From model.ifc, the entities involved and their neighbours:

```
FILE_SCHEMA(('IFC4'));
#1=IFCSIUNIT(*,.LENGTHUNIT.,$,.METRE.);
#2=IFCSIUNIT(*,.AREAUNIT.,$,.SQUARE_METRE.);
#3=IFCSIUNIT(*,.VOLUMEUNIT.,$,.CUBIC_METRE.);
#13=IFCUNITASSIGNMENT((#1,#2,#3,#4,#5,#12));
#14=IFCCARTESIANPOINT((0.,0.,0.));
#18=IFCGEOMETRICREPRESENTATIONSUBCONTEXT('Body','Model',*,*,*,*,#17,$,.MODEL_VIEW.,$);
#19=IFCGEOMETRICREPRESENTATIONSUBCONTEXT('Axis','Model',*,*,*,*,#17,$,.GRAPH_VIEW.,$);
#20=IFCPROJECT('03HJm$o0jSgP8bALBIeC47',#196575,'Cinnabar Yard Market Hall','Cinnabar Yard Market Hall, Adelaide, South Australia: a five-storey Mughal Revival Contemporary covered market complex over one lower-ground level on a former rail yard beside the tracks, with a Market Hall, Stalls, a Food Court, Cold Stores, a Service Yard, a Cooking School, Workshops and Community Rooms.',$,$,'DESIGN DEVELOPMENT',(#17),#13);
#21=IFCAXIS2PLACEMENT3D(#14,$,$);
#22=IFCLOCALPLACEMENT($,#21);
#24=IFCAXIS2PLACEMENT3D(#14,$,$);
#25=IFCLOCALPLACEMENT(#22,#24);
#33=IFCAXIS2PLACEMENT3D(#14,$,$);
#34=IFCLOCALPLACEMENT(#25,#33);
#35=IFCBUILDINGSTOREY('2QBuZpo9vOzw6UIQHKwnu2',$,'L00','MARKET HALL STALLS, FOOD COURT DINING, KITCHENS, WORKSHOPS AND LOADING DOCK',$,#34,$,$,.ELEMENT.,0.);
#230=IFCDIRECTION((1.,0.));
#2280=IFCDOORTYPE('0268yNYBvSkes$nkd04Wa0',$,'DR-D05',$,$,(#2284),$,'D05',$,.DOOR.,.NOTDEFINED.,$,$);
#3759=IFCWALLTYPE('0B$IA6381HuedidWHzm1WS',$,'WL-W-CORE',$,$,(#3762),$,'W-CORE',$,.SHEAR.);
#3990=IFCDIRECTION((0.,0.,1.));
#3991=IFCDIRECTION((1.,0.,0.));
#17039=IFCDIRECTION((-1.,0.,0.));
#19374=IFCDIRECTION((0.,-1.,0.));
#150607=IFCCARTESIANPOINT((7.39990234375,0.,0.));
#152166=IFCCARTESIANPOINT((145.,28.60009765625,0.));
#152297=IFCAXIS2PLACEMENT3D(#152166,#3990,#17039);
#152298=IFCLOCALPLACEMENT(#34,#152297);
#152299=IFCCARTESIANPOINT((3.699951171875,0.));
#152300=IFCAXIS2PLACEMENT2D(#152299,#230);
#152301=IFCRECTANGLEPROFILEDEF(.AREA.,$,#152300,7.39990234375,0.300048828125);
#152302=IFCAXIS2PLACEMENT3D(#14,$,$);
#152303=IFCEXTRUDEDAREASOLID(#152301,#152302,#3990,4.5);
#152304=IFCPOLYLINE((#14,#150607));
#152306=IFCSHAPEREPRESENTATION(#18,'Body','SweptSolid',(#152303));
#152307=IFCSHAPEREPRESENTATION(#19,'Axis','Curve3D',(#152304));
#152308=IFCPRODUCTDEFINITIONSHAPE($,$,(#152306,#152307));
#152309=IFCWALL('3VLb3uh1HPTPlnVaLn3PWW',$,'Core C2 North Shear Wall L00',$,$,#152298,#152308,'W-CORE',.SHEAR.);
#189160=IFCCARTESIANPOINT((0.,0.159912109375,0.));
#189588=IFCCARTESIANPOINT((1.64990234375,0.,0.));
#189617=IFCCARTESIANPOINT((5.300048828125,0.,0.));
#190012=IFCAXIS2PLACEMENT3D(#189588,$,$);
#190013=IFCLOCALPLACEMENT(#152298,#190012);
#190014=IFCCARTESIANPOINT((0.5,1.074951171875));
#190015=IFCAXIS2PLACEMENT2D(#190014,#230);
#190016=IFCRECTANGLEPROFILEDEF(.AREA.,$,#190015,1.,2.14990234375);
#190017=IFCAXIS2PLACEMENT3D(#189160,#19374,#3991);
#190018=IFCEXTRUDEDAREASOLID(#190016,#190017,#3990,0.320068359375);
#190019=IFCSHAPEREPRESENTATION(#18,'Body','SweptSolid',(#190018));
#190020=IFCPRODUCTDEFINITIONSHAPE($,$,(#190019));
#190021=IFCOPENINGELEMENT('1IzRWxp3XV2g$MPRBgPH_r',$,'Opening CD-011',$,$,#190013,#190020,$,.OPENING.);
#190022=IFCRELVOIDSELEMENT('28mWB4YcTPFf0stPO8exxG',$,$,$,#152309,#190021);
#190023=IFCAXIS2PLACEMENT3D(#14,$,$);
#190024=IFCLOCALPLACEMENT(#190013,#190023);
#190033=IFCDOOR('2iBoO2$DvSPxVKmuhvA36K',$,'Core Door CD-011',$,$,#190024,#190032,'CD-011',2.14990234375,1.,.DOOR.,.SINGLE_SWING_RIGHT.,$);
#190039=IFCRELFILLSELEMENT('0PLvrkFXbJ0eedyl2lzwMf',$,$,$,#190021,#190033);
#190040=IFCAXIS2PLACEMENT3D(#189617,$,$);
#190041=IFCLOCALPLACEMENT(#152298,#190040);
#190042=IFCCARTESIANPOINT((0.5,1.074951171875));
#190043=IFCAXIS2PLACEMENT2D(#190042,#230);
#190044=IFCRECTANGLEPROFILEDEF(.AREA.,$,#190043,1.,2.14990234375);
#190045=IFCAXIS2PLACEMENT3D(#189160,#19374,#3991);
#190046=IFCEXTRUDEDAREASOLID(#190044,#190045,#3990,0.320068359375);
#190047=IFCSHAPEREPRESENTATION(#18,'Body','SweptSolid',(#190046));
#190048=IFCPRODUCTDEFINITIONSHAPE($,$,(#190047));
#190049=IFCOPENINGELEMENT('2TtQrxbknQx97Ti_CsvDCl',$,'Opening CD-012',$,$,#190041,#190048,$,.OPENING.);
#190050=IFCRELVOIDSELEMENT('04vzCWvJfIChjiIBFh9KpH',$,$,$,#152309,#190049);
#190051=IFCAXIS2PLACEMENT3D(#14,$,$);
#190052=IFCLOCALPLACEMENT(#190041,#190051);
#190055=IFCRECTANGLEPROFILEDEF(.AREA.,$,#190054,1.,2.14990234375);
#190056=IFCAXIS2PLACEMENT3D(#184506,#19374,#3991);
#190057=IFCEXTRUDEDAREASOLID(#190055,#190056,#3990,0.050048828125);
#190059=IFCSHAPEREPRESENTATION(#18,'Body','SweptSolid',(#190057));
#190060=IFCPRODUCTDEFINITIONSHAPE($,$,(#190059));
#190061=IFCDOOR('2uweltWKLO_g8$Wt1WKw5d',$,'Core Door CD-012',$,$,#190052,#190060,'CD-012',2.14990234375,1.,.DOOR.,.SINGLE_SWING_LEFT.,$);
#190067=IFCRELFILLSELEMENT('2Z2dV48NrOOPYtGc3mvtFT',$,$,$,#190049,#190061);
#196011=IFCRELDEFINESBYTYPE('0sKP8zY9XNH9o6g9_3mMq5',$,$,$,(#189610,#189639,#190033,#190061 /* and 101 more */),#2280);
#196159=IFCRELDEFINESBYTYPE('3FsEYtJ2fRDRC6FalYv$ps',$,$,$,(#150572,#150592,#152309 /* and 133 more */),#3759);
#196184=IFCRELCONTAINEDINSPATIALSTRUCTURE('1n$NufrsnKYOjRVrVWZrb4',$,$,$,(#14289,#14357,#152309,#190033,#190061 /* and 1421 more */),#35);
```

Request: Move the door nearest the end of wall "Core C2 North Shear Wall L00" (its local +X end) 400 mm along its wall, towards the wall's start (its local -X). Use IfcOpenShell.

```python
import ifcopenshell
import ifcopenshell.api.geometry
import ifcopenshell.util.placement
import ifcopenshell.util.unit

model = ifcopenshell.open("model.ifc")
unit_scale = ifcopenshell.util.unit.calculate_unit_scale(model)

door = model.by_id(190061)
opening = door.FillsVoids[0].RelatingOpeningElement
wall = opening.VoidsElements[0].RelatingBuildingElement

wall_matrix = ifcopenshell.util.placement.get_local_placement(wall.ObjectPlacement)
shift = wall_matrix[:3, 0] * -0.4 / unit_scale
before = ifcopenshell.util.placement.get_local_placement(door.ObjectPlacement)[:3, 3].copy()

# The door is placed relative to its opening, so it follows when the opening moves.
matrix = ifcopenshell.util.placement.get_local_placement(opening.ObjectPlacement)
matrix[:3, 3] += shift
ifcopenshell.api.geometry.edit_object_placement(
    model, product=opening, matrix=matrix, is_si=False, should_transform_children=True
)

after = ifcopenshell.util.placement.get_local_placement(door.ObjectPlacement)[:3, 3]
print("door moved by", (after - before).round(3) + 0.0)

model.write("model_updated.ifc")
```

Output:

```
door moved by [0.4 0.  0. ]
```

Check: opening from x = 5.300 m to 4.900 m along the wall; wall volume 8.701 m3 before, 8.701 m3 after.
